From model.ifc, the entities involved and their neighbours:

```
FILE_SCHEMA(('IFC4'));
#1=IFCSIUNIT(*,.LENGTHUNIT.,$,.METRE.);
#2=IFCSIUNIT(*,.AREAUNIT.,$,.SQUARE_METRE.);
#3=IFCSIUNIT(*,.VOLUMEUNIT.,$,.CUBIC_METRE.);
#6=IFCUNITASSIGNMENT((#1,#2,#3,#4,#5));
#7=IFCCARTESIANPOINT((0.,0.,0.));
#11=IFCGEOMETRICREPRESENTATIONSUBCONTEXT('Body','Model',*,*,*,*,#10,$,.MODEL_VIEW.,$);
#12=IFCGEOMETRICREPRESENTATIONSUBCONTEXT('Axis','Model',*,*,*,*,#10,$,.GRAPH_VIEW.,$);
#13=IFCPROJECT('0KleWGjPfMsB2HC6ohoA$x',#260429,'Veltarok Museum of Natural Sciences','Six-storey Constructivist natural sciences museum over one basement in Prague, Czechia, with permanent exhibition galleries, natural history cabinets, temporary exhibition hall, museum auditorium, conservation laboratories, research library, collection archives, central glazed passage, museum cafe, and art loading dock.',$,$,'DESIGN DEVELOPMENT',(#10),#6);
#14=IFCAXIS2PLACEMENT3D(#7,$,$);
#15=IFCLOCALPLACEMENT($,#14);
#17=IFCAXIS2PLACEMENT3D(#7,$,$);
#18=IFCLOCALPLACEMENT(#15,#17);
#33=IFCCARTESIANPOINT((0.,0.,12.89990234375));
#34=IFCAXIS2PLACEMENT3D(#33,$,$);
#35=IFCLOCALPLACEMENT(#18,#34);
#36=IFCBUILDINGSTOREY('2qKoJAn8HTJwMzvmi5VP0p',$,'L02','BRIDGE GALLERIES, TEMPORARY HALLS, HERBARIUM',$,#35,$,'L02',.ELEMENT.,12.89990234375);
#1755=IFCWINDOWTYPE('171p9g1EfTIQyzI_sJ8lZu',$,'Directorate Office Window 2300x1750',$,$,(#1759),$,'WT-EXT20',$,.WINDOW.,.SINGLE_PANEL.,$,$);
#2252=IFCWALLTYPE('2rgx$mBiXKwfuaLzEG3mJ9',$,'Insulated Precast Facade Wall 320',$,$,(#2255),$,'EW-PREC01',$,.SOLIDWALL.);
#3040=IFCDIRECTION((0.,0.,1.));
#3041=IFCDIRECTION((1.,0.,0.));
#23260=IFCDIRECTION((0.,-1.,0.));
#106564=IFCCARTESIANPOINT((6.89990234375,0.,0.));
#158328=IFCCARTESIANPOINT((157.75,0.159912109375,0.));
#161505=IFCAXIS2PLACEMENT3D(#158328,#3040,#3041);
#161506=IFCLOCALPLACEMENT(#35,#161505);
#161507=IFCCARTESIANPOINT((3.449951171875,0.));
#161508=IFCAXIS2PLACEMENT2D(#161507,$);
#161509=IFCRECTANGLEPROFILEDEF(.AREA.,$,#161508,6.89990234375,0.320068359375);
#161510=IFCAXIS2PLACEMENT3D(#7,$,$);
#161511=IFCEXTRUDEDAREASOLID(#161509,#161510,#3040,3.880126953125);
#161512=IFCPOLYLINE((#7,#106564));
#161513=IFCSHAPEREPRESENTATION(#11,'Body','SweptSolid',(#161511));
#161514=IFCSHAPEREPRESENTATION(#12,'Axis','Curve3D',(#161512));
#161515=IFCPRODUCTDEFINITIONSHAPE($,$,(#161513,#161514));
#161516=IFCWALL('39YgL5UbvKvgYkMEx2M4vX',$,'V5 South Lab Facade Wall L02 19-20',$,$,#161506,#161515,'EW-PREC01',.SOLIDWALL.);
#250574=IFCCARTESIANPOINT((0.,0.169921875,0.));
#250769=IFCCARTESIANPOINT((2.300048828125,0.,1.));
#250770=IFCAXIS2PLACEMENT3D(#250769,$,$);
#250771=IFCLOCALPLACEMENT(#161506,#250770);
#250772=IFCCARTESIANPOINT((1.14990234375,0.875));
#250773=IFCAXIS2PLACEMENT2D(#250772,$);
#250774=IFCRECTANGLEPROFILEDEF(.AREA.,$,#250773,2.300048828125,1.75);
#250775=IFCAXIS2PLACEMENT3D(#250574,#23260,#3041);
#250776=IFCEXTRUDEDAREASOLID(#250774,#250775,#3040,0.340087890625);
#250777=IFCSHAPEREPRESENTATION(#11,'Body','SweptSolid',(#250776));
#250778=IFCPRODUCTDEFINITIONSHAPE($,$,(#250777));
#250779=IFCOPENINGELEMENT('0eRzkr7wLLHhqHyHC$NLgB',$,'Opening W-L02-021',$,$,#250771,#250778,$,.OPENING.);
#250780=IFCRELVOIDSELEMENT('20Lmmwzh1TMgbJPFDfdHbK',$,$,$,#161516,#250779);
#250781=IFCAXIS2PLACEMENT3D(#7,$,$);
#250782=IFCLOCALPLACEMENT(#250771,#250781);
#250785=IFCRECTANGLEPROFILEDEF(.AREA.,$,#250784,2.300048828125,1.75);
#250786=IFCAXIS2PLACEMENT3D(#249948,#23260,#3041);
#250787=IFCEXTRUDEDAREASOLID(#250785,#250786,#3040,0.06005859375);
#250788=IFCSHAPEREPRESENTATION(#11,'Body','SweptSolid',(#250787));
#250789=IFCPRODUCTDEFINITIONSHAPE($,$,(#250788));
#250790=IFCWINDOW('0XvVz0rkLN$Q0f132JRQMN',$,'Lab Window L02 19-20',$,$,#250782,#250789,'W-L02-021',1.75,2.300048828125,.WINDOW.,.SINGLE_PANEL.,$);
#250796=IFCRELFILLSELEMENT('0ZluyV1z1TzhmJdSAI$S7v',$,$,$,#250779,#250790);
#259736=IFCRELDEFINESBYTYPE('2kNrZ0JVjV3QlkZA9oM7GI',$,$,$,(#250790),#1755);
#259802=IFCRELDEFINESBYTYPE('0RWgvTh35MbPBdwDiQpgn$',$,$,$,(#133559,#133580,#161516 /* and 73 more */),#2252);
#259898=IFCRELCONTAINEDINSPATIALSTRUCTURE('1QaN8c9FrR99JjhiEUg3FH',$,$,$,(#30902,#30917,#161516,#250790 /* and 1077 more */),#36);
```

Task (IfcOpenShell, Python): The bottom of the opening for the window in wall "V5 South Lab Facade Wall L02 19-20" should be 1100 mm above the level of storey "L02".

```python
import numpy as np
import ifcopenshell
import ifcopenshell.api.geometry
import ifcopenshell.geom
import ifcopenshell.util.element
import ifcopenshell.util.placement
import ifcopenshell.util.shape
import ifcopenshell.util.unit

model = ifcopenshell.open("model.ifc")
unit_scale = ifcopenshell.util.unit.calculate_unit_scale(model)

window = model.by_id(250790)
opening = window.FillsVoids[0].RelatingOpeningElement
storey = ifcopenshell.util.element.get_container(window, ifc_class="IfcBuildingStorey")
level = ifcopenshell.util.placement.get_local_placement(storey.ObjectPlacement)[2, 3]

# The opening's origin need not be at the sill, so measure its lowest point.
shape = ifcopenshell.geom.create_shape(ifcopenshell.geom.settings(), opening)
bottom = ifcopenshell.util.shape.get_shape_bottom_elevation(shape, shape.geometry) / unit_scale
dz = level + 1.1 / unit_scale - bottom

shift = np.array([0.0, 0.0, dz])
# The window is placed relative to its opening, so it follows when the opening moves.
matrix = ifcopenshell.util.placement.get_local_placement(opening.ObjectPlacement)
matrix[:3, 3] += shift
ifcopenshell.api.geometry.edit_object_placement(
    model, product=opening, matrix=matrix, is_si=False, should_transform_children=True
)

print(f"moved by {dz * unit_scale:+.3f} m")

model.write("model_updated.ifc")
```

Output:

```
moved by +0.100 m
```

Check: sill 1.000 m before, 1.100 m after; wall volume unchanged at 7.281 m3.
